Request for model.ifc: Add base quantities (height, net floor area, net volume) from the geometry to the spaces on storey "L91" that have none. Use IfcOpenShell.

First a look at what the model holds.

```python
import ifcopenshell
import ifcopenshell.util.element
import ifcopenshell.util.unit

model = ifcopenshell.open("model.ifc")
print(model.schema)
for unit_type in ("LENGTHUNIT", "AREAUNIT", "VOLUMEUNIT"):
    print(unit_type, ifcopenshell.util.unit.calculate_unit_scale(model, unit_type))
storey = next(s for s in model.by_type("IfcBuildingStorey") if s.Name == "L91")
spaces = [e for e in ifcopenshell.util.element.get_decomposition(storey) if e.is_a("IfcSpace")]
for e in sorted(spaces, key=lambda e: e.id()):
    print(e.id(), e.is_a(), e.Name, list(ifcopenshell.util.element.get_psets(e, qtos_only=True)), sep=" | ")
```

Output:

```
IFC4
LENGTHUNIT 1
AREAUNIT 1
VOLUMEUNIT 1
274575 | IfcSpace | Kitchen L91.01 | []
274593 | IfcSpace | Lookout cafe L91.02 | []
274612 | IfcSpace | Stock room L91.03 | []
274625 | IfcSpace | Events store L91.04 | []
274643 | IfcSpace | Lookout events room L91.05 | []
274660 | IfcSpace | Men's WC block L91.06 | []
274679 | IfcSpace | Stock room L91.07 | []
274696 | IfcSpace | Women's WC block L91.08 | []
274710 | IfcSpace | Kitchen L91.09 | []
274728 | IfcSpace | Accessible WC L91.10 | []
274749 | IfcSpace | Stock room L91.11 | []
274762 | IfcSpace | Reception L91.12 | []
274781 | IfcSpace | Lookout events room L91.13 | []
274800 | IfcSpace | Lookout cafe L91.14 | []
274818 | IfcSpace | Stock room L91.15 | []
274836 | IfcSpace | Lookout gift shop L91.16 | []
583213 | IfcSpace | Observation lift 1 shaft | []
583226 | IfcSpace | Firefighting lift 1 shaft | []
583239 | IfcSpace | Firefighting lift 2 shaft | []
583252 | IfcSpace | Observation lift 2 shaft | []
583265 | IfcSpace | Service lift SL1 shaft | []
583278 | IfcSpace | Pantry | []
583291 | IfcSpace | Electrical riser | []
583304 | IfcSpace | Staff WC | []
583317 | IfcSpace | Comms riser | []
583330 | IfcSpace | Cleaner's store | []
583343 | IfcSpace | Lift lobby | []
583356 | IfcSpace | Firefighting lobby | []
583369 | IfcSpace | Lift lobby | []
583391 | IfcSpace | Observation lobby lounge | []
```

```python
import ifcopenshell
import ifcopenshell.api.pset
import ifcopenshell.geom
import ifcopenshell.util.element
import ifcopenshell.util.shape
import ifcopenshell.util.unit

model = ifcopenshell.open("model.ifc")
unit_scale = ifcopenshell.util.unit.calculate_unit_scale(model)
area_scale = ifcopenshell.util.unit.calculate_unit_scale(model, "AREAUNIT")
volume_scale = ifcopenshell.util.unit.calculate_unit_scale(model, "VOLUMEUNIT")
settings = ifcopenshell.geom.settings()

storey = next(s for s in model.by_type("IfcBuildingStorey") if s.Name == "L91")
spaces = [e for e in ifcopenshell.util.element.get_decomposition(storey) if e.is_a("IfcSpace")]

for e in sorted(spaces, key=lambda e: e.id()):
    if ifcopenshell.util.element.get_psets(e, qtos_only=True, should_inherit=False):
        continue
    # Geometry comes back in metres, in the element's own axes.
    shape = ifcopenshell.geom.create_shape(settings, e)
    values = {
        "Height": ifcopenshell.util.shape.get_z(shape.geometry) / unit_scale,
        "NetFloorArea": ifcopenshell.util.shape.get_footprint_area(shape.geometry) / area_scale,
        "NetVolume": ifcopenshell.util.shape.get_volume(shape.geometry) / volume_scale,
    }
    qto = ifcopenshell.api.pset.add_qto(model, product=e, name="Qto_SpaceBaseQuantities")
    ifcopenshell.api.pset.edit_qto(model, qto=qto, properties=values)
    print(e.id(), {k: round(v, 3) for k, v in values.items()})

model.write("model_rev.ifc")
```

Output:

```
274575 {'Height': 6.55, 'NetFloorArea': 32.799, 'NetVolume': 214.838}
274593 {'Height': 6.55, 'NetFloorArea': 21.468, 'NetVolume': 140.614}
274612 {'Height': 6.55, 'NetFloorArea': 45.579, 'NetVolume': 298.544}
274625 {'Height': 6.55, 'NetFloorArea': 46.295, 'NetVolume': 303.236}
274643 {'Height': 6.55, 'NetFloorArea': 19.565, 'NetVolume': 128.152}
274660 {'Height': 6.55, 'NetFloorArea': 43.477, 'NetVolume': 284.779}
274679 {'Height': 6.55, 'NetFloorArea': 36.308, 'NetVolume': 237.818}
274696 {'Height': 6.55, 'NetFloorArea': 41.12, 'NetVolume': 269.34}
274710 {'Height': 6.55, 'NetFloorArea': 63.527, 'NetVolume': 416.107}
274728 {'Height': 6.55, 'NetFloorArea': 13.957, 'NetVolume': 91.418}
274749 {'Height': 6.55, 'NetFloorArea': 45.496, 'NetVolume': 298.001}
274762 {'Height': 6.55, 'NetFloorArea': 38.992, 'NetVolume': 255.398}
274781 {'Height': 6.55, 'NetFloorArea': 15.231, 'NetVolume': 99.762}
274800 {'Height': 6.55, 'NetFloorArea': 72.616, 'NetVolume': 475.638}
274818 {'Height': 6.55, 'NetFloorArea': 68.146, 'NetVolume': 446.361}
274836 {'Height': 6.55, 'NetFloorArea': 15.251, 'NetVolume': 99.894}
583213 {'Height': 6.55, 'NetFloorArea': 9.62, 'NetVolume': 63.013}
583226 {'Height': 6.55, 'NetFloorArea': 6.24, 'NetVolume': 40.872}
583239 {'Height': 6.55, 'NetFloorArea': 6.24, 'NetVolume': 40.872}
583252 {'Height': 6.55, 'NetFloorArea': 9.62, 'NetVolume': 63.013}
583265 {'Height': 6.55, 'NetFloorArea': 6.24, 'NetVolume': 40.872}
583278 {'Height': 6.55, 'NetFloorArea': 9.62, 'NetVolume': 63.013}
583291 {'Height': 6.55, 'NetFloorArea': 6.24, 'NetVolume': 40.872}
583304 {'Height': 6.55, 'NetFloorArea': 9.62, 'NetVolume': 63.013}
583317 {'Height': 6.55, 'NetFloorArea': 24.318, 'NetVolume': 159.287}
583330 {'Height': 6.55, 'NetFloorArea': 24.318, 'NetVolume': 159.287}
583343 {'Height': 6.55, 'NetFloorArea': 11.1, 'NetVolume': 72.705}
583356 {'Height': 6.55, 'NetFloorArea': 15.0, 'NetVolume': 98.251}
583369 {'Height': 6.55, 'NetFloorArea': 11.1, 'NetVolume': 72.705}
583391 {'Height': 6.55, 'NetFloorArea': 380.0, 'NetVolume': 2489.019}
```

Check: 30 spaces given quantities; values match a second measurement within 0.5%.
